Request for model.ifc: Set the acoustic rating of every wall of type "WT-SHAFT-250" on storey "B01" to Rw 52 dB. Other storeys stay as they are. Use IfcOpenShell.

First a look at what the model holds.

```python
import ifcopenshell
import ifcopenshell.util.element

model = ifcopenshell.open("model.ifc")
print(model.schema)
storey = next(s for s in model.by_type("IfcBuildingStorey") if s.Name == "B01")
walls = [e for e in ifcopenshell.util.element.get_decomposition(storey) if e.is_a("IfcWall")]
seen = {}
for e in walls:
    element_type = ifcopenshell.util.element.get_type(e)
    key = (element_type.Name if element_type != e and element_type else None, ifcopenshell.util.element.get_pset(e, "Pset_WallCommon", "AcousticRating"))
    seen[key] = seen.get(key, 0) + 1
for (name, value), count in sorted(seen.items(), key=str):
    print(count, "x", name, "|", value)
```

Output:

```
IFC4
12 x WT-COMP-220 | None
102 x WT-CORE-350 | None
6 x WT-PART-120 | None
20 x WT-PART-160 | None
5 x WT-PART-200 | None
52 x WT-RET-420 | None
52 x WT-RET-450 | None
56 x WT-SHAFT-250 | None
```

```python
import ifcopenshell
import ifcopenshell.api.pset
import ifcopenshell.util.element

model = ifcopenshell.open("model.ifc")

storey = next(s for s in model.by_type("IfcBuildingStorey") if s.Name == "B01")
walls = [e for e in ifcopenshell.util.element.get_decomposition(storey) if e.is_a("IfcWall")]

count = 0
for e in walls:
    element_type = ifcopenshell.util.element.get_type(e)
    if element_type in (None, e) or element_type.Name != "WT-SHAFT-250":
        continue
    # add_pset returns the element's existing set when there is one.
    pset = ifcopenshell.api.pset.add_pset(model, product=e, name="Pset_WallCommon")
    ifcopenshell.api.pset.edit_pset(model, pset=pset, properties={"AcousticRating": "Rw 52 dB"})
    count += 1

print(count, "walls updated")

model.write("model_updated.ifc")
```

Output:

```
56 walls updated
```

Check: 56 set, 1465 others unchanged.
